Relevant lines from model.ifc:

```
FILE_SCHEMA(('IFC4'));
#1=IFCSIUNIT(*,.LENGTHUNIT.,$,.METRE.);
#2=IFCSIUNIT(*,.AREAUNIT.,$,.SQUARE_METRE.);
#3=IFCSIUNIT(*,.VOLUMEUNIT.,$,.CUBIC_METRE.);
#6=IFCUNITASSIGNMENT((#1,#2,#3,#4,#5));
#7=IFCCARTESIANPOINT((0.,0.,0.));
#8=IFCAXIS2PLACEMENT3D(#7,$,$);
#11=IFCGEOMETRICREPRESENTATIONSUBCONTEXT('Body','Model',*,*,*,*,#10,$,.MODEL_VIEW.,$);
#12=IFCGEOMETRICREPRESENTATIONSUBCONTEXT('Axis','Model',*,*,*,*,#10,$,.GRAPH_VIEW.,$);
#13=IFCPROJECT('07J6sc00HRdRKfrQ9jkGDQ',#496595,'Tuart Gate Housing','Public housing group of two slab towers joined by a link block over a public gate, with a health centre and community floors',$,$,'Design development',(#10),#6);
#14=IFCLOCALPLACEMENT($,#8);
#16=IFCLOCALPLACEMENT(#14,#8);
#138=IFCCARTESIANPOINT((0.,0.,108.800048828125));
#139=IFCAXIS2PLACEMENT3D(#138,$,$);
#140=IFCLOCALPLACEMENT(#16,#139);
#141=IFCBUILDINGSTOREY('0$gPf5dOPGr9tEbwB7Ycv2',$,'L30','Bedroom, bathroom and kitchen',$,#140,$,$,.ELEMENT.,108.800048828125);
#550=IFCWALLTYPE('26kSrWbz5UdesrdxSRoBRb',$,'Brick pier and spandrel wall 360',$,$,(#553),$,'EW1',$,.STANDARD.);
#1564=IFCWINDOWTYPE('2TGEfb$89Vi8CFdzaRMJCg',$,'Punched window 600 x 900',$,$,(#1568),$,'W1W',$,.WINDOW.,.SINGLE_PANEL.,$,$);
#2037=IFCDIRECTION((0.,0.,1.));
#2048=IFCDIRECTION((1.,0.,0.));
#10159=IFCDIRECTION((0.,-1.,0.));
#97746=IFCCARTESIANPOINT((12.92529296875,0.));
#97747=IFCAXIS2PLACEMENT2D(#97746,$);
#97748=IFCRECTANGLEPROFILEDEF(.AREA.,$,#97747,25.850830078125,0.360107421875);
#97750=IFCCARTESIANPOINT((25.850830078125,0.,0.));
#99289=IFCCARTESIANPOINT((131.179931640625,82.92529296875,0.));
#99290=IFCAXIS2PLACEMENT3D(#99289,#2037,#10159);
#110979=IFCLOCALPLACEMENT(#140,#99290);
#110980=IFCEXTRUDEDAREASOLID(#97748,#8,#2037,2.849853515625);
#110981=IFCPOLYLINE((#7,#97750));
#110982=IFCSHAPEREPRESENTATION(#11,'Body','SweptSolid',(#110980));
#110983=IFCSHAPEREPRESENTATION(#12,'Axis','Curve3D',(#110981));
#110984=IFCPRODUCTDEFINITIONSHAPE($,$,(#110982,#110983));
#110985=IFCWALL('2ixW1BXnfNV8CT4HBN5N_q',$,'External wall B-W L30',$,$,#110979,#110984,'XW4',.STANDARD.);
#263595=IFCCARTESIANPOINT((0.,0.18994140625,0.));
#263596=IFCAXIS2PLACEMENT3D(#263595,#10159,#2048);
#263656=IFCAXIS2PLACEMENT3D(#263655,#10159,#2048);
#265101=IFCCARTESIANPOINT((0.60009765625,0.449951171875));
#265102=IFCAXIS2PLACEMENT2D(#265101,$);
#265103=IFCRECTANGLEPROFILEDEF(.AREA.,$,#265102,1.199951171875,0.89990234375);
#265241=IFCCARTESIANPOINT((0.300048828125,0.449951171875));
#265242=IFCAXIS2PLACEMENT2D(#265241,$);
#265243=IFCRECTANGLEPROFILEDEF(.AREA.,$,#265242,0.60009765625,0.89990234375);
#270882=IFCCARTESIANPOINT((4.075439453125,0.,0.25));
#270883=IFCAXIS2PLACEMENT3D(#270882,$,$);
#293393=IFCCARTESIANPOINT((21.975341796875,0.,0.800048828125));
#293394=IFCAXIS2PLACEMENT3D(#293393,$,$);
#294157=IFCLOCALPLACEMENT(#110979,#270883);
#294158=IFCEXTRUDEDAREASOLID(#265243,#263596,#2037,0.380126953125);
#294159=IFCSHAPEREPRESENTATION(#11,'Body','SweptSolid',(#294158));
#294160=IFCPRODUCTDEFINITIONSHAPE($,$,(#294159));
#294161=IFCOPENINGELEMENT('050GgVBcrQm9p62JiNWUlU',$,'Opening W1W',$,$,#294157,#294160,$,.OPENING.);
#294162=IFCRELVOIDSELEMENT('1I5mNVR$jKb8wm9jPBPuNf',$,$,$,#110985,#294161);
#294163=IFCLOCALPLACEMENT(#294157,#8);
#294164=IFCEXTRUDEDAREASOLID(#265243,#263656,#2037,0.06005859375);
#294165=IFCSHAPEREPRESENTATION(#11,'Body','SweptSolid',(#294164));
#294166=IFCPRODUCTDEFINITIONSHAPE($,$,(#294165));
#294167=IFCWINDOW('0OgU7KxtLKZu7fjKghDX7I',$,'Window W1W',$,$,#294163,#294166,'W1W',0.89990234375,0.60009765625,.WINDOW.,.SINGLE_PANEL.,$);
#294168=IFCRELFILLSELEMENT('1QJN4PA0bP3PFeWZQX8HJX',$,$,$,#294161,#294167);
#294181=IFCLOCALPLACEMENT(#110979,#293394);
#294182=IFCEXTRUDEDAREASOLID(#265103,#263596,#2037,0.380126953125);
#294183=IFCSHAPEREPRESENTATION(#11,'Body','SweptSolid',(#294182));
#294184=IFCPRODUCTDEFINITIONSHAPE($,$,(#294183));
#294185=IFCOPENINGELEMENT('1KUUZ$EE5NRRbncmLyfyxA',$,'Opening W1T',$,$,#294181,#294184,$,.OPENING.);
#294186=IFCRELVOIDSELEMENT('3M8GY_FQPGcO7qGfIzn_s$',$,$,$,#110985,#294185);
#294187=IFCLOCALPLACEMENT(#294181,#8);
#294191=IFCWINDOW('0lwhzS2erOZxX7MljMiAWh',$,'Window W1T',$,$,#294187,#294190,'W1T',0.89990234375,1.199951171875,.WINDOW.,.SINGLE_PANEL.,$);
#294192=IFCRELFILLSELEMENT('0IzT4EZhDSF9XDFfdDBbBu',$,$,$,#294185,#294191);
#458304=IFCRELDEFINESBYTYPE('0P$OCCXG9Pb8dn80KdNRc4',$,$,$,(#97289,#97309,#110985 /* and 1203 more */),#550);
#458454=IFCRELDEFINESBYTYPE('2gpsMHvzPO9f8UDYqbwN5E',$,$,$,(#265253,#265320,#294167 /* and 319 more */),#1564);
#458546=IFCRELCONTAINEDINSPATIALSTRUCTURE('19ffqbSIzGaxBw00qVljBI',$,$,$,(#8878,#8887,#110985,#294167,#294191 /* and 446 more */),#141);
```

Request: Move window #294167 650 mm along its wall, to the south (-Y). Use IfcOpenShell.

```python
import ifcopenshell
import ifcopenshell.api.geometry
import ifcopenshell.util.placement
import ifcopenshell.util.unit

model = ifcopenshell.open("model.ifc")
unit_scale = ifcopenshell.util.unit.calculate_unit_scale(model)

window = model.by_id(294167)
opening = window.FillsVoids[0].RelatingOpeningElement
wall = opening.VoidsElements[0].RelatingBuildingElement

wall_matrix = ifcopenshell.util.placement.get_local_placement(wall.ObjectPlacement)
shift = wall_matrix[:3, 0] * 0.65 / unit_scale
before = ifcopenshell.util.placement.get_local_placement(window.ObjectPlacement)[:3, 3].copy()

# The window is placed relative to its opening, so it follows when the opening moves.
matrix = ifcopenshell.util.placement.get_local_placement(opening.ObjectPlacement)
matrix[:3, 3] += shift
ifcopenshell.api.geometry.edit_object_placement(
    model, product=opening, matrix=matrix, is_si=False, should_transform_children=True
)

after = ifcopenshell.util.placement.get_local_placement(window.ObjectPlacement)[:3, 3]
print("window moved by", (after - before).round(3) + 0.0)

model.write("model-out.ifc")
```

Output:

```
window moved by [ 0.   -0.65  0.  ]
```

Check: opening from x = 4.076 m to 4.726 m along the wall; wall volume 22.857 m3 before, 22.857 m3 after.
